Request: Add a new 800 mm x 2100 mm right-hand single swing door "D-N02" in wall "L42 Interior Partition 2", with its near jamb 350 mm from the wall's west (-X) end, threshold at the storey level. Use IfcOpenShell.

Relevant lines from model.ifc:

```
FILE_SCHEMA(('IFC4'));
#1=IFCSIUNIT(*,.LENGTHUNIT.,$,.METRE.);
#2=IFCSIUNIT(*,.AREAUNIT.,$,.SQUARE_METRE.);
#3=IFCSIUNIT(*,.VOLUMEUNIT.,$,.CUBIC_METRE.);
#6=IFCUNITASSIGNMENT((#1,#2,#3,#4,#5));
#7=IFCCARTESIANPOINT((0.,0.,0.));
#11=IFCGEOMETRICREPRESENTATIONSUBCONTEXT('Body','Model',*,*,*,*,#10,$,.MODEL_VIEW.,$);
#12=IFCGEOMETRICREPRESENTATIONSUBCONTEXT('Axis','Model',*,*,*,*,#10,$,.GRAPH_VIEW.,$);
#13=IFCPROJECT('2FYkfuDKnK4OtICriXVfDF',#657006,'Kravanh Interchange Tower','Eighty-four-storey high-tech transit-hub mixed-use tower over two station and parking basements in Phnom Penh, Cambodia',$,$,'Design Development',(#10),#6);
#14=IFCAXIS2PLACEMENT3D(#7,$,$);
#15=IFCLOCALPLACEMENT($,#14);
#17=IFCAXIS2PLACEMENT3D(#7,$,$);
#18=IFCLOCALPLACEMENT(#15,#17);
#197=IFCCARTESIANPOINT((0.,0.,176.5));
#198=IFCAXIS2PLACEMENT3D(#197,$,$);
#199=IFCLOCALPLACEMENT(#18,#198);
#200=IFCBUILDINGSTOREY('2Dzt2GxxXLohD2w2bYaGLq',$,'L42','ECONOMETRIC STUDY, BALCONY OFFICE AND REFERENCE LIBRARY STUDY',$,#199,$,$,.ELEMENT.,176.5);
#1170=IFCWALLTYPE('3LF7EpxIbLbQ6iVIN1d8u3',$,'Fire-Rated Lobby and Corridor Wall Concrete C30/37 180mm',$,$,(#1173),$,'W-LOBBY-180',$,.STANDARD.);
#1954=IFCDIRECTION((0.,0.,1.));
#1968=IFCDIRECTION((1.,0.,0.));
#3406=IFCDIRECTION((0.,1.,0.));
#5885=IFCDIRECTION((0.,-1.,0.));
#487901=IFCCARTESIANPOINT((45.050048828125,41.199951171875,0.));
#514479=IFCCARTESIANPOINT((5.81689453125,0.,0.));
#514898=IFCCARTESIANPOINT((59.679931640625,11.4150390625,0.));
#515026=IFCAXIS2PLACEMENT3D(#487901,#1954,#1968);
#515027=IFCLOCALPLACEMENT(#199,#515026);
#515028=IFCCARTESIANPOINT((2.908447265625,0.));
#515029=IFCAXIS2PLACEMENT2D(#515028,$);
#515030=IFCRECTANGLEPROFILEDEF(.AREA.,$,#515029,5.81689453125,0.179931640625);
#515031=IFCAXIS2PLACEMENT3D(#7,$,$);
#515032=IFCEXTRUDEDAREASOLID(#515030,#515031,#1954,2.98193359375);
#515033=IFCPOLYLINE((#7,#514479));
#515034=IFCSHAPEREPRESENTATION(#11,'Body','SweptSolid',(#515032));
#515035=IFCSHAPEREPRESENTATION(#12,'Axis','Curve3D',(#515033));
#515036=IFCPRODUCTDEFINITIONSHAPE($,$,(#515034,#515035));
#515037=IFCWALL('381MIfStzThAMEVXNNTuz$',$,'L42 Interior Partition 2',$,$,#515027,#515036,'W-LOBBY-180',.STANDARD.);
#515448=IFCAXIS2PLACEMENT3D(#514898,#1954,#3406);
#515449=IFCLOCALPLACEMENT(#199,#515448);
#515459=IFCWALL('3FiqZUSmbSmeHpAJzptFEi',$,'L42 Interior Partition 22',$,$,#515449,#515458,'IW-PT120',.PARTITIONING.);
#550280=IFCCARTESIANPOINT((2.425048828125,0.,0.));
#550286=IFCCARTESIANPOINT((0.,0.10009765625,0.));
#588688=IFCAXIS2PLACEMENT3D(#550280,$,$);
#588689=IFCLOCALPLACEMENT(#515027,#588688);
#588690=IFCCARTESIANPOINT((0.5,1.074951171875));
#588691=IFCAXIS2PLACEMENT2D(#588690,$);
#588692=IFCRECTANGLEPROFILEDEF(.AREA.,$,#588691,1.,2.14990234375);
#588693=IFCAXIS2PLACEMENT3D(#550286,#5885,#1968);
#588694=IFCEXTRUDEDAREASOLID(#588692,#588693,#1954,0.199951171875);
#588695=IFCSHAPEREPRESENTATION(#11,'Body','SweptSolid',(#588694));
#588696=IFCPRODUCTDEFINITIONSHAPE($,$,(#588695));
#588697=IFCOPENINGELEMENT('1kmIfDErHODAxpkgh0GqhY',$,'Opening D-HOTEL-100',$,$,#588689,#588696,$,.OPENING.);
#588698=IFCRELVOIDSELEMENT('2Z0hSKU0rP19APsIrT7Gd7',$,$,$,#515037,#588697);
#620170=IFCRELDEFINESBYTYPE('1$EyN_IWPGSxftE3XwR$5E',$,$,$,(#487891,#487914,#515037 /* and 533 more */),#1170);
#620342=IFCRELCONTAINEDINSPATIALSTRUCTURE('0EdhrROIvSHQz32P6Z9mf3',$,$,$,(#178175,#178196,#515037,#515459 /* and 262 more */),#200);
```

```python
import numpy as np
import ifcopenshell
import ifcopenshell.api.feature
import ifcopenshell.api.geometry
import ifcopenshell.api.root
import ifcopenshell.api.spatial
import ifcopenshell.geom
import ifcopenshell.util.element
import ifcopenshell.util.placement
import ifcopenshell.util.representation
import ifcopenshell.util.shape
import ifcopenshell.util.unit

model = ifcopenshell.open("model.ifc")
unit_scale = ifcopenshell.util.unit.calculate_unit_scale(model)
settings = ifcopenshell.geom.settings()


def volume(element):
    """Net volume in cubic metres, openings subtracted."""
    shape = ifcopenshell.geom.create_shape(settings, element)
    return ifcopenshell.util.shape.get_volume(shape.geometry)


wall = model.by_id(515037)
storey = ifcopenshell.util.element.get_container(wall, ifc_class="IfcBuildingStorey")
context = ifcopenshell.util.representation.get_context(model, "Model", "Body", "MODEL_VIEW")
before = volume(wall)

width, height, from_end, sill = 0.8, 2.1, 0.35, 0.0  # metres

# The wall runs along its own X axis, and the end named is its -X end.
wall_shape = ifcopenshell.geom.create_shape(settings, wall)
x, y, z = ifcopenshell.util.shape.get_vertices(wall_shape.geometry).T
start = x.min() + from_end
face, thickness = float(y.min()), float(y.max() - y.min())
wall_matrix = ifcopenshell.util.placement.get_local_placement(wall.ObjectPlacement)
level = ifcopenshell.util.placement.get_local_placement(storey.ObjectPlacement)[2, 3]


def in_wall(x, y):
    """Placement at x, y metres in the wall's axes, at sill height."""
    matrix = wall_matrix.copy()
    matrix[:, 3] = wall_matrix @ np.array([x / unit_scale, y / unit_scale, 0.0, 1.0])
    matrix[2, 3] = level + sill / unit_scale
    return matrix


# Opening: a box that overshoots both wall faces by 50 mm.
opening = ifcopenshell.api.root.create_entity(model, ifc_class="IfcOpeningElement", predefined_type="OPENING")
box = ifcopenshell.api.geometry.add_wall_representation(
    model, context=context, length=width, height=height, thickness=thickness + 0.1
)
ifcopenshell.api.geometry.assign_representation(model, product=opening, representation=box)
ifcopenshell.api.geometry.edit_object_placement(model, product=opening, matrix=in_wall(start, face - 0.05), is_si=False)
ifcopenshell.api.feature.add_feature(model, feature=opening, element=wall)

door = ifcopenshell.api.root.create_entity(model, ifc_class="IfcDoor", name="D-N02", predefined_type="DOOR")
door.OverallWidth, door.OverallHeight = width / unit_scale, height / unit_scale
door.OperationType = "SINGLE_SWING_RIGHT"
body = ifcopenshell.api.geometry.add_door_representation(
    model,
    context=context,
    overall_width=door.OverallWidth,
    overall_height=door.OverallHeight,
    operation_type="SINGLE_SWING_RIGHT",
    lining_properties={"LiningDepth": thickness / unit_scale, "ThresholdDepth": thickness / unit_scale},
)
ifcopenshell.api.geometry.assign_representation(model, product=door, representation=body)
ifcopenshell.api.spatial.assign_container(model, products=[door], relating_structure=storey)
ifcopenshell.api.feature.add_filling(model, opening=opening, element=door)

# The lining spans the wall, so the door starts at the wall face.
ifcopenshell.api.geometry.edit_object_placement(model, product=door, matrix=in_wall(start, face), is_si=False)

after = volume(wall)

print(f"wall volume {before:.3f} -> {after:.3f} m3")

model.write("model_rev.ifc")
```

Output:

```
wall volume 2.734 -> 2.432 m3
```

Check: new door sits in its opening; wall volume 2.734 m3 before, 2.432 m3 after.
